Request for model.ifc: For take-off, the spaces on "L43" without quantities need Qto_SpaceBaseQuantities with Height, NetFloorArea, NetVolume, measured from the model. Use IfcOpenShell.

First a look at what the model holds.

```python
import ifcopenshell
import ifcopenshell.util.element
import ifcopenshell.util.unit

model = ifcopenshell.open("model.ifc")
print(model.schema)
for unit_type in ("LENGTHUNIT", "AREAUNIT", "VOLUMEUNIT"):
    print(unit_type, ifcopenshell.util.unit.calculate_unit_scale(model, unit_type))
storey = next(s for s in model.by_type("IfcBuildingStorey") if s.Name == "L43")
spaces = [e for e in ifcopenshell.util.element.get_decomposition(storey) if e.is_a("IfcSpace")]
for e in sorted(spaces, key=lambda e: e.id()):
    print(e.id(), e.is_a(), e.Name, list(ifcopenshell.util.element.get_psets(e, qtos_only=True)), sep=" | ")
```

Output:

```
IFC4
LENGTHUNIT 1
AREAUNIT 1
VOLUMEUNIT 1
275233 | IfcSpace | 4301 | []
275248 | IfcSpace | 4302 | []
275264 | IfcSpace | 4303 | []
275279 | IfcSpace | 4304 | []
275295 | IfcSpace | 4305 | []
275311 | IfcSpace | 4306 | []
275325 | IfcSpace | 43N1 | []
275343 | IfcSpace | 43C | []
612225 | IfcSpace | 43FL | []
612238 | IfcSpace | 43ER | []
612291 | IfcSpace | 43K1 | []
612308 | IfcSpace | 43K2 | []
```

```python
import ifcopenshell
import ifcopenshell.api.pset
import ifcopenshell.geom
import ifcopenshell.util.element
import ifcopenshell.util.shape
import ifcopenshell.util.unit

model = ifcopenshell.open("model.ifc")
unit_scale = ifcopenshell.util.unit.calculate_unit_scale(model)
area_scale = ifcopenshell.util.unit.calculate_unit_scale(model, "AREAUNIT")
volume_scale = ifcopenshell.util.unit.calculate_unit_scale(model, "VOLUMEUNIT")
settings = ifcopenshell.geom.settings()

storey = next(s for s in model.by_type("IfcBuildingStorey") if s.Name == "L43")
spaces = [e for e in ifcopenshell.util.element.get_decomposition(storey) if e.is_a("IfcSpace")]

for e in sorted(spaces, key=lambda e: e.id()):
    if ifcopenshell.util.element.get_psets(e, qtos_only=True, should_inherit=False):
        continue
    # Geometry comes back in metres, in the element's own axes.
    shape = ifcopenshell.geom.create_shape(settings, e)
    values = {
        "Height": ifcopenshell.util.shape.get_z(shape.geometry) / unit_scale,
        "NetFloorArea": ifcopenshell.util.shape.get_footprint_area(shape.geometry) / area_scale,
        "NetVolume": ifcopenshell.util.shape.get_volume(shape.geometry) / volume_scale,
    }
    qto = ifcopenshell.api.pset.add_qto(model, product=e, name="Qto_SpaceBaseQuantities")
    ifcopenshell.api.pset.edit_qto(model, qto=qto, properties=values)
    print(e.id(), {k: round(v, 3) for k, v in values.items()})

model.write("model_rev.ifc")
```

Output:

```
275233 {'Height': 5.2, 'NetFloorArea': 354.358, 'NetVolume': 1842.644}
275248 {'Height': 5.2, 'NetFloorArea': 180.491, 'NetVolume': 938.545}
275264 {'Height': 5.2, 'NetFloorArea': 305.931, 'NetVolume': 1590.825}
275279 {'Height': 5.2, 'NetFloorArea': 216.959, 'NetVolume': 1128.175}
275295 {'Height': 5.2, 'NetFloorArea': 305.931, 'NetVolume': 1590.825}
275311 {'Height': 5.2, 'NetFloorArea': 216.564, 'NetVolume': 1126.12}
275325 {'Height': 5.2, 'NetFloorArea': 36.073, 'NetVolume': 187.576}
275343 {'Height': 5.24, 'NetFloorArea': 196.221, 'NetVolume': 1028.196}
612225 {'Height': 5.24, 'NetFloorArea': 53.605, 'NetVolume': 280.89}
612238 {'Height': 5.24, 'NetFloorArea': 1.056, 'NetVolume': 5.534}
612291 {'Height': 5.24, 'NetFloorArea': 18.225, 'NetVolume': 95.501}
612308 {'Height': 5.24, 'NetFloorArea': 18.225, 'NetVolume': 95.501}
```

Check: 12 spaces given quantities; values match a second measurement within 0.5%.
